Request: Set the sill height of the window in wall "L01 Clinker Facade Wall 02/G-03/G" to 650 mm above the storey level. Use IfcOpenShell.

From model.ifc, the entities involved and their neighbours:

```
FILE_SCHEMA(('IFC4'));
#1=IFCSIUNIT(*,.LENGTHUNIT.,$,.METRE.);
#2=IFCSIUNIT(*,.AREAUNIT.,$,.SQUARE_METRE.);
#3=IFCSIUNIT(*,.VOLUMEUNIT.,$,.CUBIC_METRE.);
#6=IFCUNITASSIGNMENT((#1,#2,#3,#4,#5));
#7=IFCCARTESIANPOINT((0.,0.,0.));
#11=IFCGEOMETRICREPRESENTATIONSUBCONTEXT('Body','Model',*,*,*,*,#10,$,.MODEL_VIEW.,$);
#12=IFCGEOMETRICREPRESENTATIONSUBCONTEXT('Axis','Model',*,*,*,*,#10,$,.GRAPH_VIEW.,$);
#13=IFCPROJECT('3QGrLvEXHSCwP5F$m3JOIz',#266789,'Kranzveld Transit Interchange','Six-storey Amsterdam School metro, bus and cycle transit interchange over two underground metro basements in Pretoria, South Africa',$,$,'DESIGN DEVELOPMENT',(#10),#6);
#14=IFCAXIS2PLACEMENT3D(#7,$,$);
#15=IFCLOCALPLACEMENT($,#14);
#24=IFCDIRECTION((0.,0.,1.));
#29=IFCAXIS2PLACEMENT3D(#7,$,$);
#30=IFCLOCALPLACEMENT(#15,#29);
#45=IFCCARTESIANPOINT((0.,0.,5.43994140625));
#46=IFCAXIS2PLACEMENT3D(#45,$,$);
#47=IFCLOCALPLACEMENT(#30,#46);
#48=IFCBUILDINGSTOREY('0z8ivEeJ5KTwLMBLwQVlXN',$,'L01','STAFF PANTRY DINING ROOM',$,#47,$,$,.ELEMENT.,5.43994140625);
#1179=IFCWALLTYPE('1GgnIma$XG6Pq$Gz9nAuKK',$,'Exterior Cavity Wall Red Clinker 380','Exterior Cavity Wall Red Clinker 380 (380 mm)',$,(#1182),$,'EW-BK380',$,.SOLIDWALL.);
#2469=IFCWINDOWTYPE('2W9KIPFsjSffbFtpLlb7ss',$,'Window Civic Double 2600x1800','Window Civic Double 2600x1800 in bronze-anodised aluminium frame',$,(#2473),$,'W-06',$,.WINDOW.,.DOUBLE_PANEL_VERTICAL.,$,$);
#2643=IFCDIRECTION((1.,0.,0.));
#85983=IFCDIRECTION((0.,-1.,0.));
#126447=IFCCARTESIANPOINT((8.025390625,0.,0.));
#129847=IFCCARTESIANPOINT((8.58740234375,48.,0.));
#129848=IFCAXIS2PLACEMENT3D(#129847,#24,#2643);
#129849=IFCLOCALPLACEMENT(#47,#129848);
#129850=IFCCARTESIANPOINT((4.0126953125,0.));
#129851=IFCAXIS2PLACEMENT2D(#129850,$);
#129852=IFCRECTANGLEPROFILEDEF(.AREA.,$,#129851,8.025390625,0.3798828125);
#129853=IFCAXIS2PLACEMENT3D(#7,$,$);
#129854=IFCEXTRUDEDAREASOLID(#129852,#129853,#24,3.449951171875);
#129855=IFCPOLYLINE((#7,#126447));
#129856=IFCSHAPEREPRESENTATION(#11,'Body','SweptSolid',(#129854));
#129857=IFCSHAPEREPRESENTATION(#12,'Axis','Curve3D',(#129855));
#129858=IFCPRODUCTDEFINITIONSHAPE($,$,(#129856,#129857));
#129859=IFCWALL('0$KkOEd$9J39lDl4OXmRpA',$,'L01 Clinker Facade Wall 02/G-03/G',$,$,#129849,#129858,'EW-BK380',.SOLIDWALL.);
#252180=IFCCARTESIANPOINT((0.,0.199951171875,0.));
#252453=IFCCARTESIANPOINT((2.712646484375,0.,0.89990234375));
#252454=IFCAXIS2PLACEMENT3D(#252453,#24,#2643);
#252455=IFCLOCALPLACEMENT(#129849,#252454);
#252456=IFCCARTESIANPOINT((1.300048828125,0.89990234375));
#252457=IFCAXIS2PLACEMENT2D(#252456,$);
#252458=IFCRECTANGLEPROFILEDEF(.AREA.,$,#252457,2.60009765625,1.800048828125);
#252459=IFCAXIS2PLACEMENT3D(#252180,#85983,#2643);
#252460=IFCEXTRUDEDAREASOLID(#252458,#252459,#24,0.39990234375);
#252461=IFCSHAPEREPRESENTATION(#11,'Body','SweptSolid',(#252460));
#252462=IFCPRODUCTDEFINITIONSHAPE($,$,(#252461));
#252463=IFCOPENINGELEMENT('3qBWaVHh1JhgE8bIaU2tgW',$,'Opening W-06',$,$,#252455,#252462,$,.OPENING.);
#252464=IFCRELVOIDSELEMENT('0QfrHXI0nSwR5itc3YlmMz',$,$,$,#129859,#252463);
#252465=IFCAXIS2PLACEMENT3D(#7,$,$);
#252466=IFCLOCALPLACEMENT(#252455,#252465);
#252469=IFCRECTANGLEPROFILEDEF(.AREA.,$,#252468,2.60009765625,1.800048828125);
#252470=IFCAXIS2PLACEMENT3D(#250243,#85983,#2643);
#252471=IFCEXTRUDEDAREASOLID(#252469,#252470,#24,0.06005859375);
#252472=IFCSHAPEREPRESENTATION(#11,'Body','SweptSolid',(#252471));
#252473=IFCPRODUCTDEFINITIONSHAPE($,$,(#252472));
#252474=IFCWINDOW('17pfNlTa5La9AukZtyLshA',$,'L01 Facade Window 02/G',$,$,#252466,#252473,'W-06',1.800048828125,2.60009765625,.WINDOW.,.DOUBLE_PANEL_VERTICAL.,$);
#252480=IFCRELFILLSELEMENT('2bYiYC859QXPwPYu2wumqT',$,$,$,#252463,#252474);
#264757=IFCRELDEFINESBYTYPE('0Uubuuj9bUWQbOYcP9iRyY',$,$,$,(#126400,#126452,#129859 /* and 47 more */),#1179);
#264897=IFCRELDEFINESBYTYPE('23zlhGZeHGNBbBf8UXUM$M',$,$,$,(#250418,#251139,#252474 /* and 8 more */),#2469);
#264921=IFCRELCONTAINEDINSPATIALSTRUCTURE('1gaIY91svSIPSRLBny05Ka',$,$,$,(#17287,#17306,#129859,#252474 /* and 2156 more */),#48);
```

```python
import numpy as np
import ifcopenshell
import ifcopenshell.api.geometry
import ifcopenshell.geom
import ifcopenshell.util.element
import ifcopenshell.util.placement
import ifcopenshell.util.shape
import ifcopenshell.util.unit

model = ifcopenshell.open("model.ifc")
unit_scale = ifcopenshell.util.unit.calculate_unit_scale(model)

window = model.by_id(252474)
opening = window.FillsVoids[0].RelatingOpeningElement
storey = ifcopenshell.util.element.get_container(window, ifc_class="IfcBuildingStorey")
level = ifcopenshell.util.placement.get_local_placement(storey.ObjectPlacement)[2, 3]

# The opening's origin need not be at the sill, so measure its lowest point.
shape = ifcopenshell.geom.create_shape(ifcopenshell.geom.settings(), opening)
bottom = ifcopenshell.util.shape.get_shape_bottom_elevation(shape, shape.geometry) / unit_scale
dz = level + 0.65 / unit_scale - bottom

shift = np.array([0.0, 0.0, dz])
# The window is placed relative to its opening, so it follows when the opening moves.
matrix = ifcopenshell.util.placement.get_local_placement(opening.ObjectPlacement)
matrix[:3, 3] += shift
ifcopenshell.api.geometry.edit_object_placement(
    model, product=opening, matrix=matrix, is_si=False, should_transform_children=True
)

print(f"moved by {dz * unit_scale:+.3f} m")

model.write("model_rev.ifc")
```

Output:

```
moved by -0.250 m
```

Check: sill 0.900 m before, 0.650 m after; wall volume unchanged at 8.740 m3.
